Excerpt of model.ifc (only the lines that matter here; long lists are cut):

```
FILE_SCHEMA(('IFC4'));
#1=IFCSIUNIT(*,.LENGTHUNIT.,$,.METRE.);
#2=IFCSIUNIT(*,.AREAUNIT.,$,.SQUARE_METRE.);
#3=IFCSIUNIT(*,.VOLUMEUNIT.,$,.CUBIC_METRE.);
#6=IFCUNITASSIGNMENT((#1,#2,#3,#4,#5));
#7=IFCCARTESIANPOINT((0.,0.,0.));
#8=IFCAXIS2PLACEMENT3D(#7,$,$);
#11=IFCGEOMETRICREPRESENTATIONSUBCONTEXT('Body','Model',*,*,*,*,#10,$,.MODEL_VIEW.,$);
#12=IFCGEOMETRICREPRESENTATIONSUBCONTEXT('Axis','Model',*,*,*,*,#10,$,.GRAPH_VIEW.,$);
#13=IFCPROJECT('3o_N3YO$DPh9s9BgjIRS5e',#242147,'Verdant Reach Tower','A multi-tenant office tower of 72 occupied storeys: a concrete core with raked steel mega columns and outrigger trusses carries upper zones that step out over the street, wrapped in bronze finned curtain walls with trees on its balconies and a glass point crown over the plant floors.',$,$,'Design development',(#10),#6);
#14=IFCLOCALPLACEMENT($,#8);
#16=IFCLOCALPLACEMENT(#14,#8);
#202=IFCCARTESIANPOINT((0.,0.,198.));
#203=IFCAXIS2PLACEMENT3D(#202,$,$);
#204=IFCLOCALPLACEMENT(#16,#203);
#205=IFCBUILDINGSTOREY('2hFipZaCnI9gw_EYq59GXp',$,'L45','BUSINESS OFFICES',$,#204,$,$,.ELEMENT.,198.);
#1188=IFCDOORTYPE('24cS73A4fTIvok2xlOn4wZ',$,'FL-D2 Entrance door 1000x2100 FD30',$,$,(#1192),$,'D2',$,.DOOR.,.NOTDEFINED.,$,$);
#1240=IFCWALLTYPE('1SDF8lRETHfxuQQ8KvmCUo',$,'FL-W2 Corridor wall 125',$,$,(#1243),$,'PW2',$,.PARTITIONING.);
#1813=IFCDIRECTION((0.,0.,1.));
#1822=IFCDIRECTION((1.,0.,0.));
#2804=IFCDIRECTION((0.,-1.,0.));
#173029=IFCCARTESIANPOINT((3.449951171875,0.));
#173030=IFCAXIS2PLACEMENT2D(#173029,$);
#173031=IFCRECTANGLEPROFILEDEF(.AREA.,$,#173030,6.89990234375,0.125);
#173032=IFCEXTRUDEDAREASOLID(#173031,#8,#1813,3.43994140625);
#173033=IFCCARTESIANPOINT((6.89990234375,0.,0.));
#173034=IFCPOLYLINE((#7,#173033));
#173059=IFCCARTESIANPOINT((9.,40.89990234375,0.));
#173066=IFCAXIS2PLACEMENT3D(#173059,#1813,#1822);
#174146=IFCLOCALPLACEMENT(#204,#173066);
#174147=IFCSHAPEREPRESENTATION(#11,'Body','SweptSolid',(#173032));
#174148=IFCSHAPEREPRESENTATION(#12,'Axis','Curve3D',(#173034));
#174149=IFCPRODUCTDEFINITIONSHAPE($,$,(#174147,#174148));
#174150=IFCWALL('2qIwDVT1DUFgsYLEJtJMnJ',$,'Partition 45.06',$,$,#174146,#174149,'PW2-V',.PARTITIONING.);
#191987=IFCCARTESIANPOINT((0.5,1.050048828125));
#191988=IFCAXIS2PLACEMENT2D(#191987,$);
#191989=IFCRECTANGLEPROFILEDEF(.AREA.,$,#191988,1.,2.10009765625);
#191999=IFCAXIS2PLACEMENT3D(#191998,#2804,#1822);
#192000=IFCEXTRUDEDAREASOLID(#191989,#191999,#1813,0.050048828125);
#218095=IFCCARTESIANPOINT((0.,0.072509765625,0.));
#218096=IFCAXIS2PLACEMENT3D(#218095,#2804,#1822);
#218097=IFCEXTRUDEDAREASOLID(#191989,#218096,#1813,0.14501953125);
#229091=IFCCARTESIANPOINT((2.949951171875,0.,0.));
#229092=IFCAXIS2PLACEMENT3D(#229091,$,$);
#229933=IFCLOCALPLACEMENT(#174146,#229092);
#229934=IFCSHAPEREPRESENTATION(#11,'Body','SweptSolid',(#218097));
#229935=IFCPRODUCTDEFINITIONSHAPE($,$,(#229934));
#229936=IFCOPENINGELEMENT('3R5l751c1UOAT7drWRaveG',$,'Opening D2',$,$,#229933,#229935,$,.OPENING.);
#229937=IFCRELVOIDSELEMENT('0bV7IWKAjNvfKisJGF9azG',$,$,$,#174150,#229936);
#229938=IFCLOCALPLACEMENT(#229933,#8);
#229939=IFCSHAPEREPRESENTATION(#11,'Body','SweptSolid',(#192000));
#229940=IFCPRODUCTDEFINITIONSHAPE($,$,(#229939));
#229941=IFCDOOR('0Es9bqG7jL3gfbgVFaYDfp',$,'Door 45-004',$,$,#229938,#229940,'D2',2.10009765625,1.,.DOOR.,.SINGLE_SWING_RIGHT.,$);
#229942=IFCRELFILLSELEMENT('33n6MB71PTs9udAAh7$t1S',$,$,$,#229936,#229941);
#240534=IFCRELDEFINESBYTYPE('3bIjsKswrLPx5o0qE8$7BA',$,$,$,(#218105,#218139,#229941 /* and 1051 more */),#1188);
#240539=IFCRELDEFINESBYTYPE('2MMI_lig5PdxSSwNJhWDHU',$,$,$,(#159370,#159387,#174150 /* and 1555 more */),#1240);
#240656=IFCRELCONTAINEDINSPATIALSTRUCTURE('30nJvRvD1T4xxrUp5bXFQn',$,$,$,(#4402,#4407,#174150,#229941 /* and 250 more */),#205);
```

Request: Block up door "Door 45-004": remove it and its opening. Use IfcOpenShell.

```python
import ifcopenshell
import ifcopenshell.api.feature
import ifcopenshell.api.root
import ifcopenshell.geom
import ifcopenshell.util.shape

model = ifcopenshell.open("model.ifc")
settings = ifcopenshell.geom.settings()


def volume(element):
    """Net volume in cubic metres, openings subtracted."""
    shape = ifcopenshell.geom.create_shape(settings, element)
    return ifcopenshell.util.shape.get_volume(shape.geometry)


door = model.by_guid("0Es9bqG7jL3gfbgVFaYDfp")
opening = door.FillsVoids[0].RelatingOpeningElement
wall = opening.VoidsElements[0].RelatingBuildingElement
before = volume(wall)

ifcopenshell.api.root.remove_product(model, product=door)
ifcopenshell.api.feature.remove_feature(model, feature=opening)

after = volume(wall)

print(f"wall volume {before:.3f} -> {after:.3f} m3")

model.write("model-out.ifc")
```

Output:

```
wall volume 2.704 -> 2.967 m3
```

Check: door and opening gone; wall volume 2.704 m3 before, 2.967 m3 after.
